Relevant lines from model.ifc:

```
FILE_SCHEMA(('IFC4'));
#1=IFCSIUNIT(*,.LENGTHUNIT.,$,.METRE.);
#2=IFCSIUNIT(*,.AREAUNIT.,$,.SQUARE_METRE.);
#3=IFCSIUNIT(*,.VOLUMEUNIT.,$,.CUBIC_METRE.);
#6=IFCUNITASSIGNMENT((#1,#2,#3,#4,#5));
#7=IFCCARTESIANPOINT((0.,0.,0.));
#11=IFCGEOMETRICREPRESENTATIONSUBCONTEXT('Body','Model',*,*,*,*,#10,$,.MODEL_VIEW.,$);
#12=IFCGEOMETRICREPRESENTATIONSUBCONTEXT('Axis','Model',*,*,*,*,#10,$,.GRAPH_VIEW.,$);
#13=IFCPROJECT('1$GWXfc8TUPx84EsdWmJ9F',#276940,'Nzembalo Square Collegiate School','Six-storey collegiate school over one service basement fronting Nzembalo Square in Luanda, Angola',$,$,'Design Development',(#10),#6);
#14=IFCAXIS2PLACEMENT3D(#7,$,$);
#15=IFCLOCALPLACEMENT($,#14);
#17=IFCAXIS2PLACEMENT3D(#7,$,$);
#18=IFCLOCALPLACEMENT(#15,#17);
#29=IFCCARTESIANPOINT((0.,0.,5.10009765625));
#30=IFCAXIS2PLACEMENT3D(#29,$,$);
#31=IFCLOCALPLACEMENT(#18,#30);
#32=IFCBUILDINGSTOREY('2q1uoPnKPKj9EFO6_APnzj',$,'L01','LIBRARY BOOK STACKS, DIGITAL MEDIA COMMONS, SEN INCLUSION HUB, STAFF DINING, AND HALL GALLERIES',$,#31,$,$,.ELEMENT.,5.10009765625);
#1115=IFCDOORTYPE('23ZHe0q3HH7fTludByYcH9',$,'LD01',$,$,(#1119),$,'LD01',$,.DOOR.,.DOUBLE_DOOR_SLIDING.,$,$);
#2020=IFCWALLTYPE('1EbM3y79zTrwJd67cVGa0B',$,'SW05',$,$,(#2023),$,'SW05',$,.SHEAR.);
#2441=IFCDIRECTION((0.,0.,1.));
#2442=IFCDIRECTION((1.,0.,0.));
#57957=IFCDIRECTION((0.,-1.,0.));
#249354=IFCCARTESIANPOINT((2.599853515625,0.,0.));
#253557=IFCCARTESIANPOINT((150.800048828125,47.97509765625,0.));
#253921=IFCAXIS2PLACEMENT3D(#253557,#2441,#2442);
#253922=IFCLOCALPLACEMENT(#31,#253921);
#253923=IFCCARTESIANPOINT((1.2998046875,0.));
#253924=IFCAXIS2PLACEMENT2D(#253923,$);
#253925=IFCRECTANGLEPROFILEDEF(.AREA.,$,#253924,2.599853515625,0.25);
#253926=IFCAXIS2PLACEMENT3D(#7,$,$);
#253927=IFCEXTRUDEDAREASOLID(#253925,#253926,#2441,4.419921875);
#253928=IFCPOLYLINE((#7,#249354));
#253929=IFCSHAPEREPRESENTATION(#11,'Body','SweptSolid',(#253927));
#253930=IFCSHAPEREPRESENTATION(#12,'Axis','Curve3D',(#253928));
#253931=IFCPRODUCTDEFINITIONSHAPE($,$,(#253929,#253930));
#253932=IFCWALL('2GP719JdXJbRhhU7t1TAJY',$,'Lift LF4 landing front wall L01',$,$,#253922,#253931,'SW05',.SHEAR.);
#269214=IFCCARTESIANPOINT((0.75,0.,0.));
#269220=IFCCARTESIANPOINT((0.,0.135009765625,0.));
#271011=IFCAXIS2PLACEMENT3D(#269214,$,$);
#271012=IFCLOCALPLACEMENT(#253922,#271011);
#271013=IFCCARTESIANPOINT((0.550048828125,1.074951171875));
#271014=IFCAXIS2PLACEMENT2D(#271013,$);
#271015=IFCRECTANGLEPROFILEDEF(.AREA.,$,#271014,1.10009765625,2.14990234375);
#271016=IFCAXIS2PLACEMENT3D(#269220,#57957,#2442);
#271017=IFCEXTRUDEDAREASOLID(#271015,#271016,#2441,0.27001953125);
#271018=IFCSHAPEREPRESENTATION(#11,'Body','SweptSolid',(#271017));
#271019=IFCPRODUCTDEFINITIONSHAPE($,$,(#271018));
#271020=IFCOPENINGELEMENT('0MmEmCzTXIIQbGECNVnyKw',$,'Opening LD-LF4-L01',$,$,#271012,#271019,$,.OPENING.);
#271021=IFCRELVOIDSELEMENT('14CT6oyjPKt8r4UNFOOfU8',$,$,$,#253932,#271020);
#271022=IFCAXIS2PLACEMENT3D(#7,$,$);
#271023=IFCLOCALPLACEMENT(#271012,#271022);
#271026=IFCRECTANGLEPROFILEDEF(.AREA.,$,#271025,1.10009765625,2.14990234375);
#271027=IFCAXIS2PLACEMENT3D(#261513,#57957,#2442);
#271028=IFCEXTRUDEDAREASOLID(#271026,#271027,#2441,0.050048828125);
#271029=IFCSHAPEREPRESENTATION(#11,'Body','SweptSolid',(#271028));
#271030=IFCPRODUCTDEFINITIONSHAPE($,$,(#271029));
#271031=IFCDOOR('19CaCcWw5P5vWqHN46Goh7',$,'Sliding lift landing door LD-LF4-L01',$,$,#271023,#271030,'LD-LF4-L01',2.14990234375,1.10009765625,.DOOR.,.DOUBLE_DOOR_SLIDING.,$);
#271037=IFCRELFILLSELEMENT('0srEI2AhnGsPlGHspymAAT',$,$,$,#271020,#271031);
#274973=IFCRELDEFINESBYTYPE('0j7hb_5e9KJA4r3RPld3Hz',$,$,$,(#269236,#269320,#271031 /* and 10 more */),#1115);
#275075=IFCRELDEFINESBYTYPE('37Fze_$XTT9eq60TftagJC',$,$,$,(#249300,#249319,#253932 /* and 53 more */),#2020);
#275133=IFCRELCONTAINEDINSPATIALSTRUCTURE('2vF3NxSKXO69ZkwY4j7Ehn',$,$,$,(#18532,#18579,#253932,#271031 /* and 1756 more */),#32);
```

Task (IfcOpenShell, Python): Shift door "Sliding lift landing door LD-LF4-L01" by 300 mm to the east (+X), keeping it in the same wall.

```python
import ifcopenshell
import ifcopenshell.api.geometry
import ifcopenshell.util.placement

model = ifcopenshell.open("model.ifc")

door = model.by_id(271031)
opening = door.FillsVoids[0].RelatingOpeningElement
wall = opening.VoidsElements[0].RelatingBuildingElement

wall_matrix = ifcopenshell.util.placement.get_local_placement(wall.ObjectPlacement)
shift = wall_matrix[:3, 0] * 0.3
before = ifcopenshell.util.placement.get_local_placement(door.ObjectPlacement)[:3, 3].copy()

# The door is placed relative to its opening, so it follows when the opening moves.
matrix = ifcopenshell.util.placement.get_local_placement(opening.ObjectPlacement)
matrix[:3, 3] += shift
ifcopenshell.api.geometry.edit_object_placement(
    model, product=opening, matrix=matrix, is_si=False, should_transform_children=True
)

after = ifcopenshell.util.placement.get_local_placement(door.ObjectPlacement)[:3, 3]
print("door moved by", (after - before).round(3) + 0.0)

model.write("model-out.ifc")
```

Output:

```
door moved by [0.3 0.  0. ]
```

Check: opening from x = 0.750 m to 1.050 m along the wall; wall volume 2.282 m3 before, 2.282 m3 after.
